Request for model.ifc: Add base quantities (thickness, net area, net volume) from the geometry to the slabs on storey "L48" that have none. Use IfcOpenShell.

First a look at what the model holds.

```python
import ifcopenshell
import ifcopenshell.util.element
import ifcopenshell.util.unit

model = ifcopenshell.open("model.ifc")
print(model.schema)
for unit_type in ("LENGTHUNIT", "AREAUNIT", "VOLUMEUNIT"):
    print(unit_type, ifcopenshell.util.unit.calculate_unit_scale(model, unit_type))
storey = next(s for s in model.by_type("IfcBuildingStorey") if s.Name == "L48")
slabs = [e for e in ifcopenshell.util.element.get_decomposition(storey) if e.is_a("IfcSlab")]
for e in sorted(slabs, key=lambda e: e.id()):
    print(e.id(), e.is_a(), e.Name, list(ifcopenshell.util.element.get_psets(e, qtos_only=True)), sep=" | ")
```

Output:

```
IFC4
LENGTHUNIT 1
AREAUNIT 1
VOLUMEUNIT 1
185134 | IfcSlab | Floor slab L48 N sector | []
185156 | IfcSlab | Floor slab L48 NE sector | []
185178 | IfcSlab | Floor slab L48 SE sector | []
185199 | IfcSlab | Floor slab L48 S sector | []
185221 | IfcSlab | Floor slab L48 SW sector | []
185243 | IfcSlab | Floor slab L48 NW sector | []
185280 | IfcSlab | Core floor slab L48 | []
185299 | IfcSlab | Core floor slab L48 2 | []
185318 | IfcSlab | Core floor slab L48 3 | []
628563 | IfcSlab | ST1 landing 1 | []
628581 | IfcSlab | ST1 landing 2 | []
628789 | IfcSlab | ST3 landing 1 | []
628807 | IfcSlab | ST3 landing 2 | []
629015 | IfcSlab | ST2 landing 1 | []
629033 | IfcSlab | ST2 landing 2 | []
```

```python
import ifcopenshell
import ifcopenshell.api.pset
import ifcopenshell.geom
import ifcopenshell.util.element
import ifcopenshell.util.shape
import ifcopenshell.util.unit

model = ifcopenshell.open("model.ifc")
unit_scale = ifcopenshell.util.unit.calculate_unit_scale(model)
area_scale = ifcopenshell.util.unit.calculate_unit_scale(model, "AREAUNIT")
volume_scale = ifcopenshell.util.unit.calculate_unit_scale(model, "VOLUMEUNIT")
settings = ifcopenshell.geom.settings()

storey = next(s for s in model.by_type("IfcBuildingStorey") if s.Name == "L48")
slabs = [e for e in ifcopenshell.util.element.get_decomposition(storey) if e.is_a("IfcSlab")]

for e in sorted(slabs, key=lambda e: e.id()):
    if ifcopenshell.util.element.get_psets(e, qtos_only=True, should_inherit=False):
        continue
    # Geometry comes back in metres, in the element's own axes.
    shape = ifcopenshell.geom.create_shape(settings, e)
    values = {
        "Width": ifcopenshell.util.shape.get_z(shape.geometry) / unit_scale,
        "NetArea": ifcopenshell.util.shape.get_footprint_area(shape.geometry) / area_scale,
        "NetVolume": ifcopenshell.util.shape.get_volume(shape.geometry) / volume_scale,
    }
    qto = ifcopenshell.api.pset.add_qto(model, product=e, name="Qto_SlabBaseQuantities")
    ifcopenshell.api.pset.edit_qto(model, qto=qto, properties=values)
    print(e.id(), {k: round(v, 3) for k, v in values.items()})

model.write("model_updated.ifc")
```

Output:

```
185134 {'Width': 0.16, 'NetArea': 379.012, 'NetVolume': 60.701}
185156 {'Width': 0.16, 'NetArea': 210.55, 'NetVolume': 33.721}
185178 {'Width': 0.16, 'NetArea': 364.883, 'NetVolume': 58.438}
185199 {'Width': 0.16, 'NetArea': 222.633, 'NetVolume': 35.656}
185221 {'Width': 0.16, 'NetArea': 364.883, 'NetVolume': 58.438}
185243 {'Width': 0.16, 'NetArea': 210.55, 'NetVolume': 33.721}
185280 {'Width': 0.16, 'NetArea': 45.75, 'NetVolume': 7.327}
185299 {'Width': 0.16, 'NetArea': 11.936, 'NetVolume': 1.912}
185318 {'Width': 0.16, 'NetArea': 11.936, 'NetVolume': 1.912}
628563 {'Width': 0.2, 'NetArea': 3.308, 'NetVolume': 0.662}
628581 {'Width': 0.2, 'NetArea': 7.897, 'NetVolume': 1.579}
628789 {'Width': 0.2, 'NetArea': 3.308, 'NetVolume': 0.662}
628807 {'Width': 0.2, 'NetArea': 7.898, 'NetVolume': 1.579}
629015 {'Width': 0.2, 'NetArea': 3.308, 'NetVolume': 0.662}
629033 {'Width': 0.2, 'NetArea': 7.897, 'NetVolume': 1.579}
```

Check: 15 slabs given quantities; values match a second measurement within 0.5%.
